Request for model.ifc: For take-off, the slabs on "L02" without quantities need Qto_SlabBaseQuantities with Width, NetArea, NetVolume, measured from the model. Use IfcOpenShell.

First a look at what the model holds.

```python
import ifcopenshell
import ifcopenshell.util.element
import ifcopenshell.util.unit

model = ifcopenshell.open("model.ifc")
print(model.schema)
for unit_type in ("LENGTHUNIT", "AREAUNIT", "VOLUMEUNIT"):
    print(unit_type, ifcopenshell.util.unit.calculate_unit_scale(model, unit_type))
storey = next(s for s in model.by_type("IfcBuildingStorey") if s.Name == "L02")
slabs = [e for e in ifcopenshell.util.element.get_decomposition(storey) if e.is_a("IfcSlab")]
for e in sorted(slabs, key=lambda e: e.id()):
    print(e.id(), e.is_a(), e.Name, list(ifcopenshell.util.element.get_psets(e, qtos_only=True)), sep=" | ")
```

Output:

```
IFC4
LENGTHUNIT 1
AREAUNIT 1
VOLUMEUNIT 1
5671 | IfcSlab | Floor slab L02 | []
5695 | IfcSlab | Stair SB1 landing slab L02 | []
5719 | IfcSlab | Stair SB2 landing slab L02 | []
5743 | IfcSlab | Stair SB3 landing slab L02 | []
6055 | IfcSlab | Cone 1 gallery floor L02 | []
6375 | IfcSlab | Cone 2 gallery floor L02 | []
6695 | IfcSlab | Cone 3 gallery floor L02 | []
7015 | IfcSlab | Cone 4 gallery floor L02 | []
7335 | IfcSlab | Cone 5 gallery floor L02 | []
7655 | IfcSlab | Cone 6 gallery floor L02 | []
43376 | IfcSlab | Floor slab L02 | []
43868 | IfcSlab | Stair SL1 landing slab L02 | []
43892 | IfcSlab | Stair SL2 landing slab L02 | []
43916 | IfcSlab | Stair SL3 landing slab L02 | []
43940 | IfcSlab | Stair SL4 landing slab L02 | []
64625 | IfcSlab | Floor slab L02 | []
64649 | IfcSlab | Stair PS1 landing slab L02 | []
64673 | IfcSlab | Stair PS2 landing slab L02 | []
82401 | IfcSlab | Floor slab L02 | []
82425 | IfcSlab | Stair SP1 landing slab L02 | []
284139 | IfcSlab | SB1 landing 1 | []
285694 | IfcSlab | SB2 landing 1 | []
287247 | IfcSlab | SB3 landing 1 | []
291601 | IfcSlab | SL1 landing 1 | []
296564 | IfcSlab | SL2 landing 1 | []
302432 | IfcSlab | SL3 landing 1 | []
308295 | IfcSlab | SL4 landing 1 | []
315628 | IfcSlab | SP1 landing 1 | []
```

```python
import ifcopenshell
import ifcopenshell.api.pset
import ifcopenshell.geom
import ifcopenshell.util.element
import ifcopenshell.util.shape
import ifcopenshell.util.unit

model = ifcopenshell.open("model.ifc")
unit_scale = ifcopenshell.util.unit.calculate_unit_scale(model)
area_scale = ifcopenshell.util.unit.calculate_unit_scale(model, "AREAUNIT")
volume_scale = ifcopenshell.util.unit.calculate_unit_scale(model, "VOLUMEUNIT")
settings = ifcopenshell.geom.settings()

storey = next(s for s in model.by_type("IfcBuildingStorey") if s.Name == "L02")
slabs = [e for e in ifcopenshell.util.element.get_decomposition(storey) if e.is_a("IfcSlab")]

for e in sorted(slabs, key=lambda e: e.id()):
    if ifcopenshell.util.element.get_psets(e, qtos_only=True, should_inherit=False):
        continue
    # Geometry comes back in metres, in the element's own axes.
    shape = ifcopenshell.geom.create_shape(settings, e)
    values = {
        "Width": ifcopenshell.util.shape.get_z(shape.geometry) / unit_scale,
        "NetArea": ifcopenshell.util.shape.get_footprint_area(shape.geometry) / area_scale,
        "NetVolume": ifcopenshell.util.shape.get_volume(shape.geometry) / volume_scale,
    }
    qto = ifcopenshell.api.pset.add_qto(model, product=e, name="Qto_SlabBaseQuantities")
    ifcopenshell.api.pset.edit_qto(model, qto=qto, properties=values)
    print(e.id(), {k: round(v, 3) for k, v in values.items()})

model.write("model-out.ifc")
```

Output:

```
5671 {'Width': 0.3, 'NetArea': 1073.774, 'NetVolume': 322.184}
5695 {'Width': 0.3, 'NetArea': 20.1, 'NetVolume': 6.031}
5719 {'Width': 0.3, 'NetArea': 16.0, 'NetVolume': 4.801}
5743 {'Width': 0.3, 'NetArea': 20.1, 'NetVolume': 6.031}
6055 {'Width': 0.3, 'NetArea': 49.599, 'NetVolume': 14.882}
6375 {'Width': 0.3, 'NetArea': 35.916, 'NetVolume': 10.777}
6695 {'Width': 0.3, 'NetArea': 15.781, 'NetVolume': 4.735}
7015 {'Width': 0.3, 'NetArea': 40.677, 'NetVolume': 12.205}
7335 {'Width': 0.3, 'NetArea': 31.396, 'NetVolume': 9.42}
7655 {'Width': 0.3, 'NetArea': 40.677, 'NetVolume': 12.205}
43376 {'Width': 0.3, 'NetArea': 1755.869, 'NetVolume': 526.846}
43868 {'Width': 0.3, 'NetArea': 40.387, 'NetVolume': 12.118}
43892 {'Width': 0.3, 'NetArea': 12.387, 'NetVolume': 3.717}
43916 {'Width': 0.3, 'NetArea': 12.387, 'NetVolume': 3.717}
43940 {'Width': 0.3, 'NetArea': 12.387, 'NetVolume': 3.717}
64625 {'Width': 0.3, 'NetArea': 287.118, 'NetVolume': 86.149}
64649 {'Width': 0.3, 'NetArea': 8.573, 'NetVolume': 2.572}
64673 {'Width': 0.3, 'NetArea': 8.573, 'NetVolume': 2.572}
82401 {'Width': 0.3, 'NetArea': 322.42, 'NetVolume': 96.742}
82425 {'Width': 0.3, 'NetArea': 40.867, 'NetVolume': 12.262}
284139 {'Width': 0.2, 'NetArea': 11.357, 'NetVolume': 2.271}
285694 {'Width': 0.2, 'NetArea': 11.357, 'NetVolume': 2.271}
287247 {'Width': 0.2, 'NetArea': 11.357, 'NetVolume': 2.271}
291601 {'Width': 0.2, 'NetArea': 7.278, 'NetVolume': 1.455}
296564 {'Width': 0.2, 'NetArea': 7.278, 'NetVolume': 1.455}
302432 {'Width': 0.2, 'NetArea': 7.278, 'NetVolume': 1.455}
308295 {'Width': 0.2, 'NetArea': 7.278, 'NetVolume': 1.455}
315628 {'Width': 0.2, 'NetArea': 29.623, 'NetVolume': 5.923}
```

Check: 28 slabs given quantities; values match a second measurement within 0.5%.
